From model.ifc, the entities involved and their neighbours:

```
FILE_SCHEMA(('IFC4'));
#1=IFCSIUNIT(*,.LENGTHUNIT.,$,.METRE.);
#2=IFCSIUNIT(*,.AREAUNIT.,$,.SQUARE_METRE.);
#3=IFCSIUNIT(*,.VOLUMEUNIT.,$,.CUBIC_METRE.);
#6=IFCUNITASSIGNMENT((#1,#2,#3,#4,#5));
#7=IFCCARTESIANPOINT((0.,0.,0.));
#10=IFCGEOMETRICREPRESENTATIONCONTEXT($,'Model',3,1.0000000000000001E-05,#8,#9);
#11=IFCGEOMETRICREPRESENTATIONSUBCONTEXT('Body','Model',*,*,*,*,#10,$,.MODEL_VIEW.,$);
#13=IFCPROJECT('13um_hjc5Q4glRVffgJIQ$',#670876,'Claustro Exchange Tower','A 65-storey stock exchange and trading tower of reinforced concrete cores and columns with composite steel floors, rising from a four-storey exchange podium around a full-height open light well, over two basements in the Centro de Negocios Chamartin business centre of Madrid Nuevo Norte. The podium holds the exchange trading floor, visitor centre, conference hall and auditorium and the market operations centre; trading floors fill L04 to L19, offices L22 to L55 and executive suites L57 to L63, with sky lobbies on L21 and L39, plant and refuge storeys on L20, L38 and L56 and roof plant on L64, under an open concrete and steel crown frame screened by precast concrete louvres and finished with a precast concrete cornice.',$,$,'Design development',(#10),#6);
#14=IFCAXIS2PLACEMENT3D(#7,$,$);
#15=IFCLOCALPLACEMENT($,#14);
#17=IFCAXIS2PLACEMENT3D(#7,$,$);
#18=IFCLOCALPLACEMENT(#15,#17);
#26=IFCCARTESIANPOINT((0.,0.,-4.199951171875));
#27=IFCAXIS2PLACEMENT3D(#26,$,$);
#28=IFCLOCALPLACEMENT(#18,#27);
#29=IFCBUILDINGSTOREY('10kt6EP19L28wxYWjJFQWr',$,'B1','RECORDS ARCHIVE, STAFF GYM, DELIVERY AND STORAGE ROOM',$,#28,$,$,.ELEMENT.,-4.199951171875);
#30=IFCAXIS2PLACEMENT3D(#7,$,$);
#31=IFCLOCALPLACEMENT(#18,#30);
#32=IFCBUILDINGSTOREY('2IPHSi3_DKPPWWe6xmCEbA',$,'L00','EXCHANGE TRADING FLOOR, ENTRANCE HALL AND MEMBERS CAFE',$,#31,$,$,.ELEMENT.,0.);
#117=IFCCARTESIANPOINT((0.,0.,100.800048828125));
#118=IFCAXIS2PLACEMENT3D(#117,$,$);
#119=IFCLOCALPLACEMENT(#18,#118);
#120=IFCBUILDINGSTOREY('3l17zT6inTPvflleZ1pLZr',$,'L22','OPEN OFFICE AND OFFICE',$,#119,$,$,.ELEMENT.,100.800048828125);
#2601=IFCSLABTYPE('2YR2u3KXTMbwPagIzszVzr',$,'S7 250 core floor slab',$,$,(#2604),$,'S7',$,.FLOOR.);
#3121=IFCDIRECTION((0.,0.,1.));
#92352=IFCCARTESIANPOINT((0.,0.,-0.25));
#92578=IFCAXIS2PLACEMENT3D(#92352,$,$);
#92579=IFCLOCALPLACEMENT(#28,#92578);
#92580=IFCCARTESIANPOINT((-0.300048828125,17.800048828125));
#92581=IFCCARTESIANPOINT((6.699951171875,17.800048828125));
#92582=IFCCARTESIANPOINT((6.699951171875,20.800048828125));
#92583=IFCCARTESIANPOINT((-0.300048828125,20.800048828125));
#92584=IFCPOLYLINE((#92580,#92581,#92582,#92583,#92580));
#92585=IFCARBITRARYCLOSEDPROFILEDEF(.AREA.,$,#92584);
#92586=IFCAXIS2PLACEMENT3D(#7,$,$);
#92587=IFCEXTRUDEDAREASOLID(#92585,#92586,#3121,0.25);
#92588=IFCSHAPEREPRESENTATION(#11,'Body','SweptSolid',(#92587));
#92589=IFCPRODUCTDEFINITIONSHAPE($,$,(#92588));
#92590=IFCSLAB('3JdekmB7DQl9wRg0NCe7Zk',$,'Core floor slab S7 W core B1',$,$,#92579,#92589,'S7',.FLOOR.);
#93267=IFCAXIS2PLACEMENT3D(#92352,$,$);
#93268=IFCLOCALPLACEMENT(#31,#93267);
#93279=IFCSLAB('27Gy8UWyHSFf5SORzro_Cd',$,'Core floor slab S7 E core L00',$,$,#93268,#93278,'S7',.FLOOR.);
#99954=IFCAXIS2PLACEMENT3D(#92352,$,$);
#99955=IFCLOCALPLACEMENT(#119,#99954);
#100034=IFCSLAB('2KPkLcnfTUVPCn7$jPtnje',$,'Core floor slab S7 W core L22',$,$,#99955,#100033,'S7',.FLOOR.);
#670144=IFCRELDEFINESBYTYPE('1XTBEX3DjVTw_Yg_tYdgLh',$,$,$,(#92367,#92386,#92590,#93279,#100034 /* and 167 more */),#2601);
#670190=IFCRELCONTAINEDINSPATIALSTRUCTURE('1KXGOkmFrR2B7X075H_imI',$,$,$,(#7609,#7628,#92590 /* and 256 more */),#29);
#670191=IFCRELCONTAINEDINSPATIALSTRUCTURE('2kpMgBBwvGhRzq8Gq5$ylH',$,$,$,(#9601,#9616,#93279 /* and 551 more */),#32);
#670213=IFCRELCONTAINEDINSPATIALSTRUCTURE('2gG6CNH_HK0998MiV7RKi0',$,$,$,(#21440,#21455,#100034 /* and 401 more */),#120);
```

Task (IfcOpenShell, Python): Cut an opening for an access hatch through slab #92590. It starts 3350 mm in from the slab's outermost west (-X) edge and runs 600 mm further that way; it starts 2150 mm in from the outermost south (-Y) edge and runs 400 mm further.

```python
import numpy as np
import ifcopenshell
import ifcopenshell.api.feature
import ifcopenshell.api.geometry
import ifcopenshell.api.root
import ifcopenshell.geom
import ifcopenshell.util.placement
import ifcopenshell.util.representation
import ifcopenshell.util.shape
import ifcopenshell.util.unit

model = ifcopenshell.open("model.ifc")
unit_scale = ifcopenshell.util.unit.calculate_unit_scale(model)
settings = ifcopenshell.geom.settings()


def volume(element):
    """Net volume in cubic metres, openings subtracted."""
    shape = ifcopenshell.geom.create_shape(settings, element)
    return ifcopenshell.util.shape.get_volume(shape.geometry)


slab = model.by_id(92590)
before = volume(slab)

# Extent in the slab's own axes, in metres. The edges named are its -X and -Y sides.
slab_shape = ifcopenshell.geom.create_shape(settings, slab)
vertices = ifcopenshell.util.shape.get_vertices(slab_shape.geometry)
x_min, y_min, bottom = vertices.min(axis=0)
top = vertices[:, 2].max()

opening = ifcopenshell.api.root.create_entity(model, ifc_class="IfcOpeningElement", name="Access hatch opening", predefined_type="OPENING")
context = ifcopenshell.util.representation.get_context(model, "Model", "Body", "MODEL_VIEW")
width, depth = 0.6, 0.4
outline = [(0.0, 0.0), (width, 0.0), (width, depth), (0.0, depth), (0.0, 0.0)]
# Overshoot both faces by 50 mm so the cut is clean.
shape = ifcopenshell.api.geometry.add_slab_representation(
    model, context=context, depth=top - bottom + 0.1, polyline=outline
)
ifcopenshell.api.geometry.assign_representation(model, product=opening, representation=shape)

matrix = ifcopenshell.util.placement.get_local_placement(slab.ObjectPlacement)
matrix[:, 3] = matrix @ np.append(np.array([x_min + 3.35, y_min + 2.15, bottom - 0.05]) / unit_scale, 1.0)
ifcopenshell.api.geometry.edit_object_placement(model, product=opening, matrix=matrix, is_si=False)
ifcopenshell.api.feature.add_feature(model, feature=opening, element=slab)

after = volume(slab)

print(f"slab volume {before:.3f} -> {after:.3f} m3")

model.write("model_updated.ifc")
```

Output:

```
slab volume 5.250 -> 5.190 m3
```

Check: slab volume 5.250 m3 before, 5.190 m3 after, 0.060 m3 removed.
